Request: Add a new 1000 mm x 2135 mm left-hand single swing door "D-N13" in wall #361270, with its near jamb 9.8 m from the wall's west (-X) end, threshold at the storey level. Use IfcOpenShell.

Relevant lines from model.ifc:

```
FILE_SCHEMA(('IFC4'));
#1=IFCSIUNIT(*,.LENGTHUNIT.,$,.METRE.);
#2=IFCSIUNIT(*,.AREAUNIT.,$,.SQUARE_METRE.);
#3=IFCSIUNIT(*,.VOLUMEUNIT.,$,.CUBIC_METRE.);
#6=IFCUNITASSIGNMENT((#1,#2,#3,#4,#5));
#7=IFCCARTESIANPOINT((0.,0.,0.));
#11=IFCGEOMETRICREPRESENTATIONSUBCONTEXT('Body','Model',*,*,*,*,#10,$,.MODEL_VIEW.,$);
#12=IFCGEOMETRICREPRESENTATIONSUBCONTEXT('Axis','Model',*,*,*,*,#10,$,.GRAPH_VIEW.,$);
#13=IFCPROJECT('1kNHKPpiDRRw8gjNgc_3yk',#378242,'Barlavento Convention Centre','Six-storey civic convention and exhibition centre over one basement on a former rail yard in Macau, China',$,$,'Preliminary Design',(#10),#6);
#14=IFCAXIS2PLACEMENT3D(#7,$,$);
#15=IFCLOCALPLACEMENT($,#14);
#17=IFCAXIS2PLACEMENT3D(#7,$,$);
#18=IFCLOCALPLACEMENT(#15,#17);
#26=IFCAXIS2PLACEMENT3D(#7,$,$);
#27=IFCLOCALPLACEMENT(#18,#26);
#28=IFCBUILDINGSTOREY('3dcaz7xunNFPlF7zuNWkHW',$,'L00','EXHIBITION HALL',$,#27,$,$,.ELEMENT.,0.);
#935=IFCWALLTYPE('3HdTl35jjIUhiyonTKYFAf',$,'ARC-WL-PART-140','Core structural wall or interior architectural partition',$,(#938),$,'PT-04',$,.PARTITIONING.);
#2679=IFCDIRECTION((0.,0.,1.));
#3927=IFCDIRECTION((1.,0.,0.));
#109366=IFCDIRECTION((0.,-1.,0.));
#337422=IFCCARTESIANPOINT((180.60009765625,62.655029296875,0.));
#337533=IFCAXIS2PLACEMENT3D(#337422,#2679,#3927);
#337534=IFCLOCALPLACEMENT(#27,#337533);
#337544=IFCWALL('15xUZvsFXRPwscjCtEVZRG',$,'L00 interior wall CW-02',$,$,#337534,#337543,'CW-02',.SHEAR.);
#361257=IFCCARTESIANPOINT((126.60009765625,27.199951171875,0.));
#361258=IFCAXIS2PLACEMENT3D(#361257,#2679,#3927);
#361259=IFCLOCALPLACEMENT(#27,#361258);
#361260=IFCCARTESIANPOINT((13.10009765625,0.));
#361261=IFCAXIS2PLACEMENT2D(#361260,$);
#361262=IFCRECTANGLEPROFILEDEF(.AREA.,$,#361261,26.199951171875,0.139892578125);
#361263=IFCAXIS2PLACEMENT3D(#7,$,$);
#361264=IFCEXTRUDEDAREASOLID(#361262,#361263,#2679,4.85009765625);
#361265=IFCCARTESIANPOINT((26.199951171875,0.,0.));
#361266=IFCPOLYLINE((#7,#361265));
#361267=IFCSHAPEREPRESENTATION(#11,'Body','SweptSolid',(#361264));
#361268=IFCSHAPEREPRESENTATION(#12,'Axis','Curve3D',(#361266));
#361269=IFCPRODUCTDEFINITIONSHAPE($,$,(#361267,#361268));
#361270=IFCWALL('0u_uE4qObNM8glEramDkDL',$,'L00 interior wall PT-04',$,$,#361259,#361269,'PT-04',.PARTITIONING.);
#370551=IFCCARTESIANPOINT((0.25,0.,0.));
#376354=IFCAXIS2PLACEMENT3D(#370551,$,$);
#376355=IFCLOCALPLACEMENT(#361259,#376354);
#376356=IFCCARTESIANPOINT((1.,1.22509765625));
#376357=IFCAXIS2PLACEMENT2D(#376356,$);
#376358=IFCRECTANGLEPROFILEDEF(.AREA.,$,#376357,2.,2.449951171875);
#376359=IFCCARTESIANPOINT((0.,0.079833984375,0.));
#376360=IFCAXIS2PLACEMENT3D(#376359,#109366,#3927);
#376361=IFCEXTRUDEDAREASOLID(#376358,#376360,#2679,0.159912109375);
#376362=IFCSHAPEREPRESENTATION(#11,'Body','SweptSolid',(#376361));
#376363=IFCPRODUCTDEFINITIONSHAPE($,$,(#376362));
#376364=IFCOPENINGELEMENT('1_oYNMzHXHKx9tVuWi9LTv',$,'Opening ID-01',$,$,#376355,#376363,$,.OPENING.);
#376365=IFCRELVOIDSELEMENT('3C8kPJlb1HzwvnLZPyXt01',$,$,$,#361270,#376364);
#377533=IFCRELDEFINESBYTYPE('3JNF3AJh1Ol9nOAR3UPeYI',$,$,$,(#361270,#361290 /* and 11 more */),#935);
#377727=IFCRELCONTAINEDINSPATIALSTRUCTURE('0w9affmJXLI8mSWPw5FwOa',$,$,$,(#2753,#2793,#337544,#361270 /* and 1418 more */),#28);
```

```python
import numpy as np
import ifcopenshell
import ifcopenshell.api.feature
import ifcopenshell.api.geometry
import ifcopenshell.api.root
import ifcopenshell.api.spatial
import ifcopenshell.geom
import ifcopenshell.util.element
import ifcopenshell.util.placement
import ifcopenshell.util.representation
import ifcopenshell.util.shape
import ifcopenshell.util.unit

model = ifcopenshell.open("model.ifc")
unit_scale = ifcopenshell.util.unit.calculate_unit_scale(model)
settings = ifcopenshell.geom.settings()


def volume(element):
    """Net volume in cubic metres, openings subtracted."""
    shape = ifcopenshell.geom.create_shape(settings, element)
    return ifcopenshell.util.shape.get_volume(shape.geometry)


wall = model.by_id(361270)
storey = ifcopenshell.util.element.get_container(wall, ifc_class="IfcBuildingStorey")
context = ifcopenshell.util.representation.get_context(model, "Model", "Body", "MODEL_VIEW")
before = volume(wall)

width, height, from_end, sill = 1, 2.135, 9.8, 0.0  # metres

# The wall runs along its own X axis, and the end named is its -X end.
wall_shape = ifcopenshell.geom.create_shape(settings, wall)
x, y, z = ifcopenshell.util.shape.get_vertices(wall_shape.geometry).T
start = x.min() + from_end
face, thickness = float(y.min()), float(y.max() - y.min())
wall_matrix = ifcopenshell.util.placement.get_local_placement(wall.ObjectPlacement)
level = ifcopenshell.util.placement.get_local_placement(storey.ObjectPlacement)[2, 3]


def in_wall(x, y):
    """Placement at x, y metres in the wall's axes, at sill height."""
    matrix = wall_matrix.copy()
    matrix[:, 3] = wall_matrix @ np.array([x / unit_scale, y / unit_scale, 0.0, 1.0])
    matrix[2, 3] = level + sill / unit_scale
    return matrix


# Opening: a box that overshoots both wall faces by 50 mm.
opening = ifcopenshell.api.root.create_entity(model, ifc_class="IfcOpeningElement", predefined_type="OPENING")
box = ifcopenshell.api.geometry.add_wall_representation(
    model, context=context, length=width, height=height, thickness=thickness + 0.1
)
ifcopenshell.api.geometry.assign_representation(model, product=opening, representation=box)
ifcopenshell.api.geometry.edit_object_placement(model, product=opening, matrix=in_wall(start, face - 0.05), is_si=False)
ifcopenshell.api.feature.add_feature(model, feature=opening, element=wall)

door = ifcopenshell.api.root.create_entity(model, ifc_class="IfcDoor", name="D-N13", predefined_type="DOOR")
door.OverallWidth, door.OverallHeight = width / unit_scale, height / unit_scale
door.OperationType = "SINGLE_SWING_LEFT"
body = ifcopenshell.api.geometry.add_door_representation(
    model,
    context=context,
    overall_width=door.OverallWidth,
    overall_height=door.OverallHeight,
    operation_type="SINGLE_SWING_LEFT",
    lining_properties={"LiningDepth": thickness / unit_scale, "ThresholdDepth": thickness / unit_scale},
)
ifcopenshell.api.geometry.assign_representation(model, product=door, representation=body)
ifcopenshell.api.spatial.assign_container(model, products=[door], relating_structure=storey)
ifcopenshell.api.feature.add_filling(model, opening=opening, element=door)

# The lining spans the wall, so the door starts at the wall face.
ifcopenshell.api.geometry.edit_object_placement(model, product=door, matrix=in_wall(start, face), is_si=False)

after = volume(wall)

print(f"wall volume {before:.3f} -> {after:.3f} m3")

model.write("model_edited.ifc")
```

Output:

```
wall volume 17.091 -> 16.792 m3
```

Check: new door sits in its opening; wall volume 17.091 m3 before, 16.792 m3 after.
